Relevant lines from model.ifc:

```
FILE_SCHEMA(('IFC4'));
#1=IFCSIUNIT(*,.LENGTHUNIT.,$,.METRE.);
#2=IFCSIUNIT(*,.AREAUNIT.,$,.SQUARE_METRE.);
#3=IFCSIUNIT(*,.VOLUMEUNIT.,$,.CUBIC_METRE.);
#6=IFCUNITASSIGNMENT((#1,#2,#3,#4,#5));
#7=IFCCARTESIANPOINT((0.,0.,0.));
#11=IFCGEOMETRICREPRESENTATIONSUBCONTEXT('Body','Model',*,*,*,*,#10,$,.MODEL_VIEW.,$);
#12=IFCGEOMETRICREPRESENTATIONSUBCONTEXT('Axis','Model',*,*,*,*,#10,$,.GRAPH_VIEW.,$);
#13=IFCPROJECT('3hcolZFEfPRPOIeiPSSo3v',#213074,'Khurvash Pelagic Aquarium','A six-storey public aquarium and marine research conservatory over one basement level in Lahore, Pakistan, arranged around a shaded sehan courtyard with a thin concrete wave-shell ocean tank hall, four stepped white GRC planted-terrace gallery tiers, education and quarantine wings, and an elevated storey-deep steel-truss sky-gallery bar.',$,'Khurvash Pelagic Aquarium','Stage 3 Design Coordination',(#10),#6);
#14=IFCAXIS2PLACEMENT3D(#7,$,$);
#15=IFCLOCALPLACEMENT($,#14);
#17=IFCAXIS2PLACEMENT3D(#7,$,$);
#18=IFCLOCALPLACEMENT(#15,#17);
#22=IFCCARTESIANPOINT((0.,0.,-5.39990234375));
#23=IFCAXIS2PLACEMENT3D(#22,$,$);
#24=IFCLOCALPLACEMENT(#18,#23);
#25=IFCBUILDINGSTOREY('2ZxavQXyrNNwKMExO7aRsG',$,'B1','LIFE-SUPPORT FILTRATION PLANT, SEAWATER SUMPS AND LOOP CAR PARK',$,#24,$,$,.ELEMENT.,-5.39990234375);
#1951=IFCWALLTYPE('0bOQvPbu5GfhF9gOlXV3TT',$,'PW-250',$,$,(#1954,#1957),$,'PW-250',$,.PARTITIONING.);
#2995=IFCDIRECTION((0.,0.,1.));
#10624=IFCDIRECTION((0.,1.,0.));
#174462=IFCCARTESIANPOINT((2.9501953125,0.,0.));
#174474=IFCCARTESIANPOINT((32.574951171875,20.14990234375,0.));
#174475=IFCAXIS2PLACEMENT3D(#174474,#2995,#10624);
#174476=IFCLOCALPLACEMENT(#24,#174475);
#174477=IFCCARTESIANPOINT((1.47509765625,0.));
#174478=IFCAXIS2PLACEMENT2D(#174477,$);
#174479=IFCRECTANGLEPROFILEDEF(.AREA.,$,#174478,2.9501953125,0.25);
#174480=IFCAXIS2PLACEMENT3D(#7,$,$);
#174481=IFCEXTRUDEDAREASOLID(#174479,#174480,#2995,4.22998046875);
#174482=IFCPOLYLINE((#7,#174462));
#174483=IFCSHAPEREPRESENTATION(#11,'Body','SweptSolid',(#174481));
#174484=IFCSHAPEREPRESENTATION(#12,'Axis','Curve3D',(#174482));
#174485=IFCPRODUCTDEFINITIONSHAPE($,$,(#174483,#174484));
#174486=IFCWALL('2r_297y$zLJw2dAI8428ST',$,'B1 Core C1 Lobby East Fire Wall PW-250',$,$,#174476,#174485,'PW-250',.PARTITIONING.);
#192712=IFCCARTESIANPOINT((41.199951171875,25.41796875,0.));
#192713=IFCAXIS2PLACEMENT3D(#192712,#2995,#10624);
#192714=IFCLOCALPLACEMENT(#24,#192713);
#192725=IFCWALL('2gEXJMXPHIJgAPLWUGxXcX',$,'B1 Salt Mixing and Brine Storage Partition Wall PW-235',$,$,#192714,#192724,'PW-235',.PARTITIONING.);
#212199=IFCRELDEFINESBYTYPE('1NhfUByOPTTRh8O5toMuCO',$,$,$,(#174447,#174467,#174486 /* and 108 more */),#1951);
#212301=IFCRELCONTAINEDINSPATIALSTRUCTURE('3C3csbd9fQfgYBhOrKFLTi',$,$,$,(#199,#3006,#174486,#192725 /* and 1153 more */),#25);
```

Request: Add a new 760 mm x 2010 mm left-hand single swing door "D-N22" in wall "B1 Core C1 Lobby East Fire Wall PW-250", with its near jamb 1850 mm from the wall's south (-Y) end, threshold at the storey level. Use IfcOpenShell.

```python
import numpy as np
import ifcopenshell
import ifcopenshell.api.feature
import ifcopenshell.api.geometry
import ifcopenshell.api.root
import ifcopenshell.api.spatial
import ifcopenshell.geom
import ifcopenshell.util.element
import ifcopenshell.util.placement
import ifcopenshell.util.representation
import ifcopenshell.util.shape
import ifcopenshell.util.unit

model = ifcopenshell.open("model.ifc")
unit_scale = ifcopenshell.util.unit.calculate_unit_scale(model)
settings = ifcopenshell.geom.settings()


def volume(element):
    """Net volume in cubic metres, openings subtracted."""
    shape = ifcopenshell.geom.create_shape(settings, element)
    return ifcopenshell.util.shape.get_volume(shape.geometry)


wall = model.by_guid("2r_297y$zLJw2dAI8428ST")
storey = ifcopenshell.util.element.get_container(wall, ifc_class="IfcBuildingStorey")
context = ifcopenshell.util.representation.get_context(model, "Model", "Body", "MODEL_VIEW")
before = volume(wall)

width, height, from_end, sill = 0.76, 2.01, 1.85, 0.0  # metres

# The wall runs along its own X axis, and the end named is its -X end.
wall_shape = ifcopenshell.geom.create_shape(settings, wall)
x, y, z = ifcopenshell.util.shape.get_vertices(wall_shape.geometry).T
start = x.min() + from_end
face, thickness = float(y.min()), float(y.max() - y.min())
wall_matrix = ifcopenshell.util.placement.get_local_placement(wall.ObjectPlacement)
level = ifcopenshell.util.placement.get_local_placement(storey.ObjectPlacement)[2, 3]


def in_wall(x, y):
    """Placement at x, y metres in the wall's axes, at sill height."""
    matrix = wall_matrix.copy()
    matrix[:, 3] = wall_matrix @ np.array([x / unit_scale, y / unit_scale, 0.0, 1.0])
    matrix[2, 3] = level + sill / unit_scale
    return matrix


# Opening: a box that overshoots both wall faces by 50 mm.
opening = ifcopenshell.api.root.create_entity(model, ifc_class="IfcOpeningElement", predefined_type="OPENING")
box = ifcopenshell.api.geometry.add_wall_representation(
    model, context=context, length=width, height=height, thickness=thickness + 0.1
)
ifcopenshell.api.geometry.assign_representation(model, product=opening, representation=box)
ifcopenshell.api.geometry.edit_object_placement(model, product=opening, matrix=in_wall(start, face - 0.05), is_si=False)
ifcopenshell.api.feature.add_feature(model, feature=opening, element=wall)

door = ifcopenshell.api.root.create_entity(model, ifc_class="IfcDoor", name="D-N22", predefined_type="DOOR")
door.OverallWidth, door.OverallHeight = width / unit_scale, height / unit_scale
door.OperationType = "SINGLE_SWING_LEFT"
body = ifcopenshell.api.geometry.add_door_representation(
    model,
    context=context,
    overall_width=door.OverallWidth,
    overall_height=door.OverallHeight,
    operation_type="SINGLE_SWING_LEFT",
    lining_properties={"LiningDepth": thickness / unit_scale, "ThresholdDepth": thickness / unit_scale},
)
ifcopenshell.api.geometry.assign_representation(model, product=door, representation=body)
ifcopenshell.api.spatial.assign_container(model, products=[door], relating_structure=storey)
ifcopenshell.api.feature.add_filling(model, opening=opening, element=door)

# The lining spans the wall, so the door starts at the wall face.
ifcopenshell.api.geometry.edit_object_placement(model, product=door, matrix=in_wall(start, face), is_si=False)

after = volume(wall)

print(f"wall volume {before:.3f} -> {after:.3f} m3")

model.write("model-out.ifc")
```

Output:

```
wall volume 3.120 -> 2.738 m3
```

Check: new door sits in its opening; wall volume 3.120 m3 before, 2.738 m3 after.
